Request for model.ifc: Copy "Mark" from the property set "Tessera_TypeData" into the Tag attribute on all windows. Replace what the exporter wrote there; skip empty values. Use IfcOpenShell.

First a look at what the model holds.

```python
import ifcopenshell
import ifcopenshell.util.element

model = ifcopenshell.open("model.ifc")
print(model.schema)
windows = model.by_type("IfcWindow")
print(len(windows), "windows")
for e in windows[:8]:
    source = ifcopenshell.util.element.get_pset(e, "Tessera_TypeData", "Mark")
    target = e.Tag
    print(e.id(), repr(source), repr(target), sep=" | ")
```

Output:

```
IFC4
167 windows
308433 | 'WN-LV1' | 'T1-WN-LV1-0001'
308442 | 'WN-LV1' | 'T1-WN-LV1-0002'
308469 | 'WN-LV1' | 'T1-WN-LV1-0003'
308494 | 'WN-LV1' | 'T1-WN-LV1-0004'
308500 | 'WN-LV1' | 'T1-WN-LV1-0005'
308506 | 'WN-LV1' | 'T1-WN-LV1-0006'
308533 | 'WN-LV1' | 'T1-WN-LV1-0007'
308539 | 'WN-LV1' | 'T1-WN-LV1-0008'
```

```python
import ifcopenshell
import ifcopenshell.util.element

model = ifcopenshell.open("model.ifc")

count = 0
for e in model.by_type("IfcWindow"):
    value = ifcopenshell.util.element.get_pset(e, "Tessera_TypeData", "Mark")
    current = e.Tag
    if not value or not value.strip() or current == value:
        continue
    e.Tag = value
    count += 1

print(count, "windows updated")

model.write("model_rev.ifc")
```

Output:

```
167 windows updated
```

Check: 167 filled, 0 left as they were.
